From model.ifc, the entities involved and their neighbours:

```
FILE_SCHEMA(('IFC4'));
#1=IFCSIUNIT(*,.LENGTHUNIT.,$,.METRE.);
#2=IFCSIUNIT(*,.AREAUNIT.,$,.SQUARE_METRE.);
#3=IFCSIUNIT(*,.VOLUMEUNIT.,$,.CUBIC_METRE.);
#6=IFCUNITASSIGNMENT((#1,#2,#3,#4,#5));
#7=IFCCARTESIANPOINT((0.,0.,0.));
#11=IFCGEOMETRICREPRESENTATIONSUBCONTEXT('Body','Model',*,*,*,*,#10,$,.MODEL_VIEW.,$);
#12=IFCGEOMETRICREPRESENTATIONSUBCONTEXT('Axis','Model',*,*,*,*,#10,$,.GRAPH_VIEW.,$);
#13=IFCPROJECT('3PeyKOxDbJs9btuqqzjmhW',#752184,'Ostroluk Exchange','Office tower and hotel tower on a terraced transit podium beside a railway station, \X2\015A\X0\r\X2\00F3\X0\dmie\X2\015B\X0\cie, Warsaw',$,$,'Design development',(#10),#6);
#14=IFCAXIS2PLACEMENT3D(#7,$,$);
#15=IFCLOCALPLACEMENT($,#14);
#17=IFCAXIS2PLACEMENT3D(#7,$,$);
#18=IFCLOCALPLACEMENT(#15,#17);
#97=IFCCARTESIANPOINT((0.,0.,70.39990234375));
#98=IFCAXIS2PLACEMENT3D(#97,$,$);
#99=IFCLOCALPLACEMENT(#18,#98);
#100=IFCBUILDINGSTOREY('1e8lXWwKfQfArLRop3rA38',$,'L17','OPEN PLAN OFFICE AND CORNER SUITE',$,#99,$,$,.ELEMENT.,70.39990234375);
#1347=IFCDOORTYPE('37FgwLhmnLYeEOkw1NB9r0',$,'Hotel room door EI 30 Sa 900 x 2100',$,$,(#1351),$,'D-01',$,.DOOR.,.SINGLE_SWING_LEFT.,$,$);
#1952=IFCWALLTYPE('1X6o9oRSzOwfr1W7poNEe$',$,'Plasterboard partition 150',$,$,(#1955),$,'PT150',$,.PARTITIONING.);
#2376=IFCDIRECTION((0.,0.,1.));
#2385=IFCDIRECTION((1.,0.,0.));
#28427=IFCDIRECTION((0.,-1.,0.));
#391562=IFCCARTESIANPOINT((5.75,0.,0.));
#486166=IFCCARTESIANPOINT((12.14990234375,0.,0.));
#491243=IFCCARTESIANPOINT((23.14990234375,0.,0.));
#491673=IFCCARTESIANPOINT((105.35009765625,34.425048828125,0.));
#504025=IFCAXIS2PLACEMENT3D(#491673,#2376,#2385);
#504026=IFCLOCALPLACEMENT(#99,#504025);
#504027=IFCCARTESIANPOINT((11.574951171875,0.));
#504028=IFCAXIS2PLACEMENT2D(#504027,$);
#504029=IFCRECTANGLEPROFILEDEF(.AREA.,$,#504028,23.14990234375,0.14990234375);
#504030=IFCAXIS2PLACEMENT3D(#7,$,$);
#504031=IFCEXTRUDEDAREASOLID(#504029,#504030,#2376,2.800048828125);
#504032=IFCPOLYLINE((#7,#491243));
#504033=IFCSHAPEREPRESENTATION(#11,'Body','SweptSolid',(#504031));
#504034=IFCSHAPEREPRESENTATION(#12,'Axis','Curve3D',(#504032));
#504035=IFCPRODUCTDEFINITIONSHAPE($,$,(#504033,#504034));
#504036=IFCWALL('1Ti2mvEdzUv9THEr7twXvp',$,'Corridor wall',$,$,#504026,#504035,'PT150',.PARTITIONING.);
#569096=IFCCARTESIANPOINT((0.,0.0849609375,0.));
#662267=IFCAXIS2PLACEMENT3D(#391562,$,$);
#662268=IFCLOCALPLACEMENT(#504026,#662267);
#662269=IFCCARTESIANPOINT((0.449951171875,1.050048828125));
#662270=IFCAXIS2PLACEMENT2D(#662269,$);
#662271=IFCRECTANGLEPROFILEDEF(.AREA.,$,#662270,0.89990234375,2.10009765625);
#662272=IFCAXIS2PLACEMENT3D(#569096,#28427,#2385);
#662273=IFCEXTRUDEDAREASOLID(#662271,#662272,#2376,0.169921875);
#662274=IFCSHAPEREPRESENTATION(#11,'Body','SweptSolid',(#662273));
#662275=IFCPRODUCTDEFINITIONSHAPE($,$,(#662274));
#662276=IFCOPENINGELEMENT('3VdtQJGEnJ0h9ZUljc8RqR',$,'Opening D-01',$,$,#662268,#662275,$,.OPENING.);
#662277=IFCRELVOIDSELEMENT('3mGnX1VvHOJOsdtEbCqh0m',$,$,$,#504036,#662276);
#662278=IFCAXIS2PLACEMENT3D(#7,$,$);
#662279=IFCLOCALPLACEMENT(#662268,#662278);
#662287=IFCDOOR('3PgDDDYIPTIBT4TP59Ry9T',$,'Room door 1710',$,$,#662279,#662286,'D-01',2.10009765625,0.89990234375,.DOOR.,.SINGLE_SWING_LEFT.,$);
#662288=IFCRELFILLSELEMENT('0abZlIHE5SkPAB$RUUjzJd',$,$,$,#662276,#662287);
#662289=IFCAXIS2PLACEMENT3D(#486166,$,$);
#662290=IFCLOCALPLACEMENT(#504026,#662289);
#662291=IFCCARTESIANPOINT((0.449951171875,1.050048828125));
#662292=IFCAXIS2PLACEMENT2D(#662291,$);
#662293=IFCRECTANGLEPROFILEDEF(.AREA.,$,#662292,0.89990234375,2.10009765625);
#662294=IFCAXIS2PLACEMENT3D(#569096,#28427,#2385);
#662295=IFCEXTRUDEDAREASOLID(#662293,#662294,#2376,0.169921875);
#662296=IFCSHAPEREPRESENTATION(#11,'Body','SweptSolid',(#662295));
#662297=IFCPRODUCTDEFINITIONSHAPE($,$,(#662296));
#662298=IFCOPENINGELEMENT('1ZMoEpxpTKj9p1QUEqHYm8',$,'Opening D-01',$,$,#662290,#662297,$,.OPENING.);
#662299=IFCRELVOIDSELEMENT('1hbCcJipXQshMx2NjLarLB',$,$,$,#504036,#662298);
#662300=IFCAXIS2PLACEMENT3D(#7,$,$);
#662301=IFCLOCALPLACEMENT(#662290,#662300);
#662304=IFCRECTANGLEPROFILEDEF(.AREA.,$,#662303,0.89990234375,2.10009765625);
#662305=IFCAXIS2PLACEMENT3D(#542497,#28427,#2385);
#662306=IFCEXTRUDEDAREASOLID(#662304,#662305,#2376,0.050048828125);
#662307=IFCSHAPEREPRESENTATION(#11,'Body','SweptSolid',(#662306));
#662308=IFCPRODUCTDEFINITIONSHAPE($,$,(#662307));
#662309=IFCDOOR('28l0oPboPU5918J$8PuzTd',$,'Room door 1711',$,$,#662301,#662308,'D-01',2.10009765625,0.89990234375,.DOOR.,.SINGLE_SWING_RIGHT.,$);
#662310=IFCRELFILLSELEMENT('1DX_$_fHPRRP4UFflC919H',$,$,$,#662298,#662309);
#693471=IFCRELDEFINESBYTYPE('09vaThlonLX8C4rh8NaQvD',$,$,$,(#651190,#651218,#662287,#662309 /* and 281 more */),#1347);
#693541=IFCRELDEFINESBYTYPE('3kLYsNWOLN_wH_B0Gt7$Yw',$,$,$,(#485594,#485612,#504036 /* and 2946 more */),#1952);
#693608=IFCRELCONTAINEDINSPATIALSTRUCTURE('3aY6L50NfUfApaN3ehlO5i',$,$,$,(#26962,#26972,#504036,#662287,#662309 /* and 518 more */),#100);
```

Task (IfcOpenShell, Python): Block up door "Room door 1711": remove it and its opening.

```python
import ifcopenshell
import ifcopenshell.api.feature
import ifcopenshell.api.root
import ifcopenshell.geom
import ifcopenshell.util.shape

model = ifcopenshell.open("model.ifc")
settings = ifcopenshell.geom.settings()


def volume(element):
    """Net volume in cubic metres, openings subtracted."""
    shape = ifcopenshell.geom.create_shape(settings, element)
    return ifcopenshell.util.shape.get_volume(shape.geometry)


door = model.by_guid("28l0oPboPU5918J$8PuzTd")
opening = door.FillsVoids[0].RelatingOpeningElement
wall = opening.VoidsElements[0].RelatingBuildingElement
before = volume(wall)

ifcopenshell.api.root.remove_product(model, product=door)
ifcopenshell.api.feature.remove_feature(model, feature=opening)

after = volume(wall)

print(f"wall volume {before:.3f} -> {after:.3f} m3")

model.write("model_updated.ifc")
```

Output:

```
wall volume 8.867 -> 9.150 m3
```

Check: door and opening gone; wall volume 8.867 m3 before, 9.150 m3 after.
